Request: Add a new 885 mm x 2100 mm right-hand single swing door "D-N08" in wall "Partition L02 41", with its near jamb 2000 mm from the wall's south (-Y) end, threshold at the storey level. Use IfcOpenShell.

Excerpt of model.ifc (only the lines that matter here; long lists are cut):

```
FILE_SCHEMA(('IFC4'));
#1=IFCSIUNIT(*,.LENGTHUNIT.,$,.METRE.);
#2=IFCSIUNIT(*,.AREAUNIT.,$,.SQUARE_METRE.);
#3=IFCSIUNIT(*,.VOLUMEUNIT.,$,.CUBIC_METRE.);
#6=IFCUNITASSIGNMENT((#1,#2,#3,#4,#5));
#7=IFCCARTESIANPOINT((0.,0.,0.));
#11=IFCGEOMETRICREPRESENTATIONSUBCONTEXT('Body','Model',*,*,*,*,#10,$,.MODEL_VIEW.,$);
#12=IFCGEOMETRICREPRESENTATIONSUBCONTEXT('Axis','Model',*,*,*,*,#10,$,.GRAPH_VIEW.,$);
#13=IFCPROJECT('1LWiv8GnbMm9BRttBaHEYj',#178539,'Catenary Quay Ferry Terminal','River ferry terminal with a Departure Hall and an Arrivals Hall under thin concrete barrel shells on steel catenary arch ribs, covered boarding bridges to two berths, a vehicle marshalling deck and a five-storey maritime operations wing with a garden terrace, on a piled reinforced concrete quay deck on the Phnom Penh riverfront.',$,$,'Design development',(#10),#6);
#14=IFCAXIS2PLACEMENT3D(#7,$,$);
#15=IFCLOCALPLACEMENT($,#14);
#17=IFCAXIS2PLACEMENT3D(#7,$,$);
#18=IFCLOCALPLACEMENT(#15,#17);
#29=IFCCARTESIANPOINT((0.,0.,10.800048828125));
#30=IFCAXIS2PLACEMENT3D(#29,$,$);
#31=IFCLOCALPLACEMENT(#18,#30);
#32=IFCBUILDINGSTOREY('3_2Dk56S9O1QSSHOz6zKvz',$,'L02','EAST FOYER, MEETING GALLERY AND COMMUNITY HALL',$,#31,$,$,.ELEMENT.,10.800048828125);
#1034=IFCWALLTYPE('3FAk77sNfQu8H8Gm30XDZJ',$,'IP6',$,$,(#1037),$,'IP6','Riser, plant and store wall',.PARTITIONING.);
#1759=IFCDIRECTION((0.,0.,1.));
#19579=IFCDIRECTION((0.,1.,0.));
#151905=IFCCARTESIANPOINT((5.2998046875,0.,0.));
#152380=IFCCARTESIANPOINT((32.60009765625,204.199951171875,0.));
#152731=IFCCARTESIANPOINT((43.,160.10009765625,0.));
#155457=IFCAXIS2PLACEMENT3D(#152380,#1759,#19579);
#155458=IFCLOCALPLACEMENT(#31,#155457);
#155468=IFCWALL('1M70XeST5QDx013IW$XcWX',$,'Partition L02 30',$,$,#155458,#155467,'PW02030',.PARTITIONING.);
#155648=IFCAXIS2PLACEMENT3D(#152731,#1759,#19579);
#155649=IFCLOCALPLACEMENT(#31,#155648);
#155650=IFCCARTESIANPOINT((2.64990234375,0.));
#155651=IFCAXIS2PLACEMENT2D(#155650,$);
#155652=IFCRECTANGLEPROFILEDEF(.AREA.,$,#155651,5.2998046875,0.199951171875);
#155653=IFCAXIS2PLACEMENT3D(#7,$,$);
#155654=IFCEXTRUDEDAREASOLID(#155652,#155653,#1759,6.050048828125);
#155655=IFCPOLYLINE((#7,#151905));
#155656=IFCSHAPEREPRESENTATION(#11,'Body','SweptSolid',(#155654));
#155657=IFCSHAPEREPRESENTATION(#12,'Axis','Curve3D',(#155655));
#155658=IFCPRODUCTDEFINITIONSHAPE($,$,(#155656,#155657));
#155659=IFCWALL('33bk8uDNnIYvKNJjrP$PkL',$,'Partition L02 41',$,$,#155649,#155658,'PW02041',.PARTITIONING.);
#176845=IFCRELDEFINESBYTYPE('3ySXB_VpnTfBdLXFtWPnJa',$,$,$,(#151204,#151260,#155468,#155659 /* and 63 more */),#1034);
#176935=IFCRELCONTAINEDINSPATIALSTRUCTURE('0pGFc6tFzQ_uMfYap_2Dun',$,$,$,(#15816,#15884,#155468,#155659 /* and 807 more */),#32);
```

```python
import numpy as np
import ifcopenshell
import ifcopenshell.api.feature
import ifcopenshell.api.geometry
import ifcopenshell.api.root
import ifcopenshell.api.spatial
import ifcopenshell.geom
import ifcopenshell.util.element
import ifcopenshell.util.placement
import ifcopenshell.util.representation
import ifcopenshell.util.shape
import ifcopenshell.util.unit

model = ifcopenshell.open("model.ifc")
unit_scale = ifcopenshell.util.unit.calculate_unit_scale(model)
settings = ifcopenshell.geom.settings()


def volume(element):
    """Net volume in cubic metres, openings subtracted."""
    shape = ifcopenshell.geom.create_shape(settings, element)
    return ifcopenshell.util.shape.get_volume(shape.geometry)


wall = model.by_guid("33bk8uDNnIYvKNJjrP$PkL")
storey = ifcopenshell.util.element.get_container(wall, ifc_class="IfcBuildingStorey")
context = ifcopenshell.util.representation.get_context(model, "Model", "Body", "MODEL_VIEW")
before = volume(wall)

width, height, from_end, sill = 0.885, 2.1, 2, 0.0  # metres

# The wall runs along its own X axis, and the end named is its -X end.
wall_shape = ifcopenshell.geom.create_shape(settings, wall)
x, y, z = ifcopenshell.util.shape.get_vertices(wall_shape.geometry).T
start = x.min() + from_end
face, thickness = float(y.min()), float(y.max() - y.min())
wall_matrix = ifcopenshell.util.placement.get_local_placement(wall.ObjectPlacement)
level = ifcopenshell.util.placement.get_local_placement(storey.ObjectPlacement)[2, 3]


def in_wall(x, y):
    """Placement at x, y metres in the wall's axes, at sill height."""
    matrix = wall_matrix.copy()
    matrix[:, 3] = wall_matrix @ np.array([x / unit_scale, y / unit_scale, 0.0, 1.0])
    matrix[2, 3] = level + sill / unit_scale
    return matrix


# Opening: a box that overshoots both wall faces by 50 mm.
opening = ifcopenshell.api.root.create_entity(model, ifc_class="IfcOpeningElement", predefined_type="OPENING")
box = ifcopenshell.api.geometry.add_wall_representation(
    model, context=context, length=width, height=height, thickness=thickness + 0.1
)
ifcopenshell.api.geometry.assign_representation(model, product=opening, representation=box)
ifcopenshell.api.geometry.edit_object_placement(model, product=opening, matrix=in_wall(start, face - 0.05), is_si=False)
ifcopenshell.api.feature.add_feature(model, feature=opening, element=wall)

door = ifcopenshell.api.root.create_entity(model, ifc_class="IfcDoor", name="D-N08", predefined_type="DOOR")
door.OverallWidth, door.OverallHeight = width / unit_scale, height / unit_scale
door.OperationType = "SINGLE_SWING_RIGHT"
body = ifcopenshell.api.geometry.add_door_representation(
    model,
    context=context,
    overall_width=door.OverallWidth,
    overall_height=door.OverallHeight,
    operation_type="SINGLE_SWING_RIGHT",
    lining_properties={"LiningDepth": thickness / unit_scale, "ThresholdDepth": thickness / unit_scale},
)
ifcopenshell.api.geometry.assign_representation(model, product=door, representation=body)
ifcopenshell.api.spatial.assign_container(model, products=[door], relating_structure=storey)
ifcopenshell.api.feature.add_filling(model, opening=opening, element=door)

# The lining spans the wall, so the door starts at the wall face.
ifcopenshell.api.geometry.edit_object_placement(model, product=door, matrix=in_wall(start, face), is_si=False)

after = volume(wall)

print(f"wall volume {before:.3f} -> {after:.3f} m3")

model.write("model-out.ifc")
```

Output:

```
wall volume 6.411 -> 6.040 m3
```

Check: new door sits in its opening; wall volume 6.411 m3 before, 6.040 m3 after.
